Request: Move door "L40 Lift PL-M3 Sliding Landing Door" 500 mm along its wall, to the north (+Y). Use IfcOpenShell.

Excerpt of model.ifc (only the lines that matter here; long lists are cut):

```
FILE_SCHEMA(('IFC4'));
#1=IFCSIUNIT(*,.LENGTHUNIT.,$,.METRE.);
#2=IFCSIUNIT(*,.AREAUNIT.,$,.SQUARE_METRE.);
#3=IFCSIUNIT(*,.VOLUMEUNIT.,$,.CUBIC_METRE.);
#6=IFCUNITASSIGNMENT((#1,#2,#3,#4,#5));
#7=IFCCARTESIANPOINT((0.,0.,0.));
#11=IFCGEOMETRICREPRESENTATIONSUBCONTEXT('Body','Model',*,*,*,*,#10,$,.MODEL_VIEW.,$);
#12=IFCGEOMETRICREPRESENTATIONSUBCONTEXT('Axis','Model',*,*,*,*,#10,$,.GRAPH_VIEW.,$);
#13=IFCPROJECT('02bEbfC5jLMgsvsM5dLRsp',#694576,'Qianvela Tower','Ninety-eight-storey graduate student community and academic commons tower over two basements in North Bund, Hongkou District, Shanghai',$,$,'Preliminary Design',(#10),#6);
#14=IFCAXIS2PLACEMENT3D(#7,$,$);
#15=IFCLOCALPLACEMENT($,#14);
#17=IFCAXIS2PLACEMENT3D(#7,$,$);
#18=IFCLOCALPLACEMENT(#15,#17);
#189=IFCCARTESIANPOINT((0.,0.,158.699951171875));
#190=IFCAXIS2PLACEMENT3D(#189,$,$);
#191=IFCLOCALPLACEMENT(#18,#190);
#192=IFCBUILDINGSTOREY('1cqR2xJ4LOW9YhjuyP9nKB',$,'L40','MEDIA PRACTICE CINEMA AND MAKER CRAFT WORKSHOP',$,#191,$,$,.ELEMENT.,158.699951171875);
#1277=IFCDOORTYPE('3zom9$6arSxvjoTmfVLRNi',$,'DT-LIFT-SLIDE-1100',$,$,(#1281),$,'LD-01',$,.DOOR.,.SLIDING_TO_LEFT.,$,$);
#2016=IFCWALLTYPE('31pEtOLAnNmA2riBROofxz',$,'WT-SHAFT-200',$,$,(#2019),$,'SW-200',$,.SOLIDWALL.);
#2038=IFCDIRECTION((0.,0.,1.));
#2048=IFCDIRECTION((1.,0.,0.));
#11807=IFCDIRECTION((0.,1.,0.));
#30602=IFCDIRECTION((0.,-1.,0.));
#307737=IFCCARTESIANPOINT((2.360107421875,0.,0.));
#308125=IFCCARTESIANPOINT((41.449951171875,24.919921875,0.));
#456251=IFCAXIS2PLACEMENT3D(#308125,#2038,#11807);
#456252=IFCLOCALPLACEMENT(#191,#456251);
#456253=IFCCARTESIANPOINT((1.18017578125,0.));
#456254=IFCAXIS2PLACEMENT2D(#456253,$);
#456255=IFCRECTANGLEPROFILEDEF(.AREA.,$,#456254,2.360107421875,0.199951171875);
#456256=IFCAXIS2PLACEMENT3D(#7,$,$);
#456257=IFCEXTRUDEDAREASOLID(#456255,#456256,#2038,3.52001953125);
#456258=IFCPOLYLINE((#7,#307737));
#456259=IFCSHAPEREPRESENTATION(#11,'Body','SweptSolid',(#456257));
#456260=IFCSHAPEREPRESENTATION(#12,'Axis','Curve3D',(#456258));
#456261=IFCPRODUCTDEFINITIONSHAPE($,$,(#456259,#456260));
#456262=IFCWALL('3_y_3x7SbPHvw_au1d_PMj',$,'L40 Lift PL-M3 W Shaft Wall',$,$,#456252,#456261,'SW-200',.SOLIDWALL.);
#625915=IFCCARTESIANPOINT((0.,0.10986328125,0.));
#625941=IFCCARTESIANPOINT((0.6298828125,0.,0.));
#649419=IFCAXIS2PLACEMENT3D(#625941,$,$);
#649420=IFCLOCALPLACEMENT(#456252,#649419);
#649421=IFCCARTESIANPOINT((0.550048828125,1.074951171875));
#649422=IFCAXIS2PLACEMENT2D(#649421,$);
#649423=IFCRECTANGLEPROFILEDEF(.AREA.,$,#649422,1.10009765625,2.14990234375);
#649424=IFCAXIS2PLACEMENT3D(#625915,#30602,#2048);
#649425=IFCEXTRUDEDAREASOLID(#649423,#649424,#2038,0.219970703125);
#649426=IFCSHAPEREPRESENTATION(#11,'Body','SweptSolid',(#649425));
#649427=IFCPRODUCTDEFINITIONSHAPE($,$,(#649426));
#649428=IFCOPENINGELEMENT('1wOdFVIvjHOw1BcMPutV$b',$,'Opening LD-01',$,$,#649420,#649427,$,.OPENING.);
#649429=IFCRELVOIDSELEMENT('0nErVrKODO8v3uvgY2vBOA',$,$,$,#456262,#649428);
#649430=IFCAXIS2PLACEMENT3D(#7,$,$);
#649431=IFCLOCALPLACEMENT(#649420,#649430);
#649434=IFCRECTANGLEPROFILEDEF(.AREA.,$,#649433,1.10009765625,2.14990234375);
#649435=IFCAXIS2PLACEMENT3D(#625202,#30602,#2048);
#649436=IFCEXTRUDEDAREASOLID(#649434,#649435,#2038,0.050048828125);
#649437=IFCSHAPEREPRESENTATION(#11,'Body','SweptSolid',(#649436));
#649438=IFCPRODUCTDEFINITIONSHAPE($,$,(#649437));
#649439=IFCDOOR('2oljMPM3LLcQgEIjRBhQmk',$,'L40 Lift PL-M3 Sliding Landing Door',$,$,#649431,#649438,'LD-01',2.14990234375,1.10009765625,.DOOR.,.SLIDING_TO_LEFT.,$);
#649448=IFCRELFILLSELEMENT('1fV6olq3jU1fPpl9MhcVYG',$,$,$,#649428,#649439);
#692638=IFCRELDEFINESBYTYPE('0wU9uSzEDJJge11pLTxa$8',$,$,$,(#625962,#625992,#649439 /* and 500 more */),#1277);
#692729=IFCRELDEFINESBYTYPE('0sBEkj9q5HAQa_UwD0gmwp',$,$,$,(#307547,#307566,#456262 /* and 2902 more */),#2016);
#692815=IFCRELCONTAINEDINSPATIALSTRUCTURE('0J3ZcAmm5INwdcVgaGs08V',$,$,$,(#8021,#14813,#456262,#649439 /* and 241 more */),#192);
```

```python
import ifcopenshell
import ifcopenshell.api.geometry
import ifcopenshell.util.placement

model = ifcopenshell.open("model.ifc")

door = model.by_guid("2oljMPM3LLcQgEIjRBhQmk")
opening = door.FillsVoids[0].RelatingOpeningElement
wall = opening.VoidsElements[0].RelatingBuildingElement

wall_matrix = ifcopenshell.util.placement.get_local_placement(wall.ObjectPlacement)
shift = wall_matrix[:3, 0] * 0.5
before = ifcopenshell.util.placement.get_local_placement(door.ObjectPlacement)[:3, 3].copy()

# The door is placed relative to its opening, so it follows when the opening moves.
matrix = ifcopenshell.util.placement.get_local_placement(opening.ObjectPlacement)
matrix[:3, 3] += shift
ifcopenshell.api.geometry.edit_object_placement(
    model, product=opening, matrix=matrix, is_si=False, should_transform_children=True
)

after = ifcopenshell.util.placement.get_local_placement(door.ObjectPlacement)[:3, 3]
print("door moved by", (after - before).round(3) + 0.0)

model.write("model_updated.ifc")
```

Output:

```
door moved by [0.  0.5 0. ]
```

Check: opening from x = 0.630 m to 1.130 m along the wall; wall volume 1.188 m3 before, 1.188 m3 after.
